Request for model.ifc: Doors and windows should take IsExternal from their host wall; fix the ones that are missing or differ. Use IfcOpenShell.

First a look at what the model holds.

```python
import ifcopenshell
import ifcopenshell.util.element

model = ifcopenshell.open("model.ifc")
print(model.schema)
seen = {}
for e in model.by_type("IfcDoor") + model.by_type("IfcWindow"):
    if not e.FillsVoids:
        continue
    host = e.FillsVoids[0].RelatingOpeningElement.VoidsElements[0].RelatingBuildingElement
    own = ifcopenshell.util.element.get_pset(e, f"Pset_{e.is_a()[3:].removesuffix('StandardCase')}Common", "IsExternal")
    wall = ifcopenshell.util.element.get_pset(host, "Pset_WallCommon", "IsExternal")
    seen[e.is_a(), own, wall] = seen.get((e.is_a(), own, wall), 0) + 1
for (cls, own, wall), count in sorted(seen.items(), key=str):
    print(count, cls, "IsExternal:", own, "| host wall:", wall)
```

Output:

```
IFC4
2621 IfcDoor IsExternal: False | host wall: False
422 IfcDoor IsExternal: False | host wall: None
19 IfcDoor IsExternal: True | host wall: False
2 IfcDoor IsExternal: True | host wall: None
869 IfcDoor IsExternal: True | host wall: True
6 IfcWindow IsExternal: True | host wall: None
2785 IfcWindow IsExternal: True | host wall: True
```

```python
import ifcopenshell
import ifcopenshell.api.pset
import ifcopenshell.util.element

model = ifcopenshell.open("model.ifc")

count = 0
for ifc_class, pset_name in (("IfcDoor", "Pset_DoorCommon"), ("IfcWindow", "Pset_WindowCommon")):
    for e in model.by_type(ifc_class):
        if not e.FillsVoids:
            continue
        host = e.FillsVoids[0].RelatingOpeningElement.VoidsElements[0].RelatingBuildingElement
        external = ifcopenshell.util.element.get_pset(host, "Pset_WallCommon", "IsExternal")
        if external is None or ifcopenshell.util.element.get_pset(e, pset_name, "IsExternal") == external:
            continue
        pset = ifcopenshell.api.pset.add_pset(model, product=e, name=pset_name)
        ifcopenshell.api.pset.edit_pset(model, pset=pset, properties={"IsExternal": external})
        count += 1

print(count, "updated")

model.write("model_edited.ifc")
```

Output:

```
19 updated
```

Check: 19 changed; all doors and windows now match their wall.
